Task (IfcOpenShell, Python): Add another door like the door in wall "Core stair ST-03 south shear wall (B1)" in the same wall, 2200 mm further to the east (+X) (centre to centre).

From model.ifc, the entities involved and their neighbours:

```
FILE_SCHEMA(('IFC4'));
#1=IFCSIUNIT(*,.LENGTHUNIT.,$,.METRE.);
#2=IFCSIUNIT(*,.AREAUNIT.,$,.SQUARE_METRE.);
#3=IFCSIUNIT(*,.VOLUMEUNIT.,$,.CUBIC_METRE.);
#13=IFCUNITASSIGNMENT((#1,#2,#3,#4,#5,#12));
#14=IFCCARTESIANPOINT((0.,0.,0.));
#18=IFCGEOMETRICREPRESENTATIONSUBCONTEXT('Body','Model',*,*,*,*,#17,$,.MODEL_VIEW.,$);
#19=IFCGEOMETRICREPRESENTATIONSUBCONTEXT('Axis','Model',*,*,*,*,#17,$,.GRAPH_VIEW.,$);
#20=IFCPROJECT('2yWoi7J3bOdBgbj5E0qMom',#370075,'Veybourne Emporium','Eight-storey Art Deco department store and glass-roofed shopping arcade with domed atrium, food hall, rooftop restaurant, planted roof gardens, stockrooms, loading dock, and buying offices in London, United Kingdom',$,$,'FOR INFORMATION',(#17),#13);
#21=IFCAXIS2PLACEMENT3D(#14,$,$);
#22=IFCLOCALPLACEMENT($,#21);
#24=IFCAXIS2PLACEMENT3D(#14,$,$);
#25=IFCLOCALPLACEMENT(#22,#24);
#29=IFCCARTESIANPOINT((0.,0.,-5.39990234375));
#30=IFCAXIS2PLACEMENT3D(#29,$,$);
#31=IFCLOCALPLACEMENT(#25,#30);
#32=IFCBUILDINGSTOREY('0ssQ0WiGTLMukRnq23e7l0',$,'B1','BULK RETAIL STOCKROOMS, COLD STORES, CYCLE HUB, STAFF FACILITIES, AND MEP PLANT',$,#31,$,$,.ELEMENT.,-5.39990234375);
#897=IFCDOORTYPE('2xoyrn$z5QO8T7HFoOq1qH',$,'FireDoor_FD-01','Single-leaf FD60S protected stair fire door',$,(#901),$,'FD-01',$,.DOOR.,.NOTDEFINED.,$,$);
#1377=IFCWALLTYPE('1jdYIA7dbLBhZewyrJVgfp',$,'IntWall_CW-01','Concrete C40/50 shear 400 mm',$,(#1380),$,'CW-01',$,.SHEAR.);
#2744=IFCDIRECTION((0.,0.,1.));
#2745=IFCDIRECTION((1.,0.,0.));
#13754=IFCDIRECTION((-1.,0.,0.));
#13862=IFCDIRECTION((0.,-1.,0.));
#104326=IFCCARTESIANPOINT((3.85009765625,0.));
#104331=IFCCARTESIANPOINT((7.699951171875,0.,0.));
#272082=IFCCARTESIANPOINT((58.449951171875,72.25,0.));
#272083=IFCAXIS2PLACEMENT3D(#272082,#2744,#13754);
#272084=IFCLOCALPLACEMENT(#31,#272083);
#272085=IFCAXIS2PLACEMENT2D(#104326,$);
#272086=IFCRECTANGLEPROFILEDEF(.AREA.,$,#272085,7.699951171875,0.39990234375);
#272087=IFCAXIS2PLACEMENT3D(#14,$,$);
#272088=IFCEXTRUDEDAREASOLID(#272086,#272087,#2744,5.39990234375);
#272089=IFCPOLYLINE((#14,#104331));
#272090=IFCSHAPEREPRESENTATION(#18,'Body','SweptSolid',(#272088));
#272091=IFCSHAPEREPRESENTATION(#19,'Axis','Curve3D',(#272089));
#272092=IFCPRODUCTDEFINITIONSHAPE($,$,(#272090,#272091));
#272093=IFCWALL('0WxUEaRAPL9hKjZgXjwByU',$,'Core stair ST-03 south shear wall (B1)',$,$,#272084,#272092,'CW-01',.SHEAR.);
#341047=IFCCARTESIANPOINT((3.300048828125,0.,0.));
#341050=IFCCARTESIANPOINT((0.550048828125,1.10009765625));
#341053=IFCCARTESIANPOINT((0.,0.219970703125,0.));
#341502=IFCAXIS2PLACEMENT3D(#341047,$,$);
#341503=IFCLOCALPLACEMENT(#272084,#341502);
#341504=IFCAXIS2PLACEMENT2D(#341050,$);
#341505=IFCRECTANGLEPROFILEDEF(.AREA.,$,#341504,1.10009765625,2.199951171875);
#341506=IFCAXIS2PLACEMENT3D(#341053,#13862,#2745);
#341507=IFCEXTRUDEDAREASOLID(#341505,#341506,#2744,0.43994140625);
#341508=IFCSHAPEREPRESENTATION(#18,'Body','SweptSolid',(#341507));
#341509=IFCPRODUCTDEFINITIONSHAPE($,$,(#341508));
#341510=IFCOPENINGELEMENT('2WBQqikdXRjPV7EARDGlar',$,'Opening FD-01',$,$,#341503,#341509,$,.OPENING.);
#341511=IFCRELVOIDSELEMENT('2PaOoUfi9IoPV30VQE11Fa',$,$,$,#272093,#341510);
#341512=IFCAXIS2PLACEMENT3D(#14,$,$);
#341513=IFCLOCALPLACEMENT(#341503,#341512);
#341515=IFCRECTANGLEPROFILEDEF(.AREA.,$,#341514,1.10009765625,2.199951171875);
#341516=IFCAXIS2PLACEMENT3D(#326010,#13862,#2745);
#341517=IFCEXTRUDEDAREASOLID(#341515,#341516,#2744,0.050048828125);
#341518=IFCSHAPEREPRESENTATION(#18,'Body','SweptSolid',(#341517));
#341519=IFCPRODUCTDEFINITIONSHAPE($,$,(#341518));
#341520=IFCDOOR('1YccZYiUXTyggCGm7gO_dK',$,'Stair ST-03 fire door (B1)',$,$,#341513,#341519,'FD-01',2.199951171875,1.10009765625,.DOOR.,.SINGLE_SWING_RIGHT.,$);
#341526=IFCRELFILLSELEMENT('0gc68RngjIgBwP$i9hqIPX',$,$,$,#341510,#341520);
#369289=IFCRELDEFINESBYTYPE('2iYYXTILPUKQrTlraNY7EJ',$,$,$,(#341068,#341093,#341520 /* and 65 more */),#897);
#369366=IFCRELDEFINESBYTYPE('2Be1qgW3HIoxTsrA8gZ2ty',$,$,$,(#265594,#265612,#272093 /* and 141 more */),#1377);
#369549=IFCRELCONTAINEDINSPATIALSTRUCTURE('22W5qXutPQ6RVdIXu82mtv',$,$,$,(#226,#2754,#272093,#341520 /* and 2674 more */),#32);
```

```python
import ifcopenshell
import ifcopenshell.api.feature
import ifcopenshell.api.geometry
import ifcopenshell.api.root
import ifcopenshell.geom
import ifcopenshell.util.element
import ifcopenshell.util.placement
import ifcopenshell.util.shape
import ifcopenshell.util.unit

model = ifcopenshell.open("model.ifc")
unit_scale = ifcopenshell.util.unit.calculate_unit_scale(model)
settings = ifcopenshell.geom.settings()


def volume(element):
    """Net volume in cubic metres, openings subtracted."""
    shape = ifcopenshell.geom.create_shape(settings, element)
    return ifcopenshell.util.shape.get_volume(shape.geometry)


door = model.by_guid("1YccZYiUXTyggCGm7gO_dK")
opening = door.FillsVoids[0].RelatingOpeningElement
wall = opening.VoidsElements[0].RelatingBuildingElement
before = volume(wall)
shift = ifcopenshell.util.placement.get_local_placement(wall.ObjectPlacement)[:3, 0] * -2.2 / unit_scale

# copy_class copies the void relationship, type, container and properties, but no geometry.
new_opening = ifcopenshell.api.root.copy_class(model, product=opening)
new_opening.Representation = ifcopenshell.util.element.copy_deep(
    model, opening.Representation, exclude=["IfcGeometricRepresentationContext", "IfcRepresentationMap"]
)
new_door = ifcopenshell.api.root.copy_class(model, product=door)
new_door.Representation = ifcopenshell.util.element.copy_deep(
    model, door.Representation, exclude=["IfcGeometricRepresentationContext", "IfcRepresentationMap"]
)
new_door.Tag = None
ifcopenshell.api.feature.add_filling(model, opening=new_opening, element=new_door)

for old, new in ((opening, new_opening), (door, new_door)):
    matrix = ifcopenshell.util.placement.get_local_placement(old.ObjectPlacement)
    matrix[:3, 3] += shift
    ifcopenshell.api.geometry.edit_object_placement(model, product=new, matrix=matrix, is_si=False)

after = volume(wall)

print(f"wall volume {before:.3f} -> {after:.3f} m3")

model.write("model_edited.ifc")
```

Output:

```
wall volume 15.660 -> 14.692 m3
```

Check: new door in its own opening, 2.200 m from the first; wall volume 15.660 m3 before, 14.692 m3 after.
